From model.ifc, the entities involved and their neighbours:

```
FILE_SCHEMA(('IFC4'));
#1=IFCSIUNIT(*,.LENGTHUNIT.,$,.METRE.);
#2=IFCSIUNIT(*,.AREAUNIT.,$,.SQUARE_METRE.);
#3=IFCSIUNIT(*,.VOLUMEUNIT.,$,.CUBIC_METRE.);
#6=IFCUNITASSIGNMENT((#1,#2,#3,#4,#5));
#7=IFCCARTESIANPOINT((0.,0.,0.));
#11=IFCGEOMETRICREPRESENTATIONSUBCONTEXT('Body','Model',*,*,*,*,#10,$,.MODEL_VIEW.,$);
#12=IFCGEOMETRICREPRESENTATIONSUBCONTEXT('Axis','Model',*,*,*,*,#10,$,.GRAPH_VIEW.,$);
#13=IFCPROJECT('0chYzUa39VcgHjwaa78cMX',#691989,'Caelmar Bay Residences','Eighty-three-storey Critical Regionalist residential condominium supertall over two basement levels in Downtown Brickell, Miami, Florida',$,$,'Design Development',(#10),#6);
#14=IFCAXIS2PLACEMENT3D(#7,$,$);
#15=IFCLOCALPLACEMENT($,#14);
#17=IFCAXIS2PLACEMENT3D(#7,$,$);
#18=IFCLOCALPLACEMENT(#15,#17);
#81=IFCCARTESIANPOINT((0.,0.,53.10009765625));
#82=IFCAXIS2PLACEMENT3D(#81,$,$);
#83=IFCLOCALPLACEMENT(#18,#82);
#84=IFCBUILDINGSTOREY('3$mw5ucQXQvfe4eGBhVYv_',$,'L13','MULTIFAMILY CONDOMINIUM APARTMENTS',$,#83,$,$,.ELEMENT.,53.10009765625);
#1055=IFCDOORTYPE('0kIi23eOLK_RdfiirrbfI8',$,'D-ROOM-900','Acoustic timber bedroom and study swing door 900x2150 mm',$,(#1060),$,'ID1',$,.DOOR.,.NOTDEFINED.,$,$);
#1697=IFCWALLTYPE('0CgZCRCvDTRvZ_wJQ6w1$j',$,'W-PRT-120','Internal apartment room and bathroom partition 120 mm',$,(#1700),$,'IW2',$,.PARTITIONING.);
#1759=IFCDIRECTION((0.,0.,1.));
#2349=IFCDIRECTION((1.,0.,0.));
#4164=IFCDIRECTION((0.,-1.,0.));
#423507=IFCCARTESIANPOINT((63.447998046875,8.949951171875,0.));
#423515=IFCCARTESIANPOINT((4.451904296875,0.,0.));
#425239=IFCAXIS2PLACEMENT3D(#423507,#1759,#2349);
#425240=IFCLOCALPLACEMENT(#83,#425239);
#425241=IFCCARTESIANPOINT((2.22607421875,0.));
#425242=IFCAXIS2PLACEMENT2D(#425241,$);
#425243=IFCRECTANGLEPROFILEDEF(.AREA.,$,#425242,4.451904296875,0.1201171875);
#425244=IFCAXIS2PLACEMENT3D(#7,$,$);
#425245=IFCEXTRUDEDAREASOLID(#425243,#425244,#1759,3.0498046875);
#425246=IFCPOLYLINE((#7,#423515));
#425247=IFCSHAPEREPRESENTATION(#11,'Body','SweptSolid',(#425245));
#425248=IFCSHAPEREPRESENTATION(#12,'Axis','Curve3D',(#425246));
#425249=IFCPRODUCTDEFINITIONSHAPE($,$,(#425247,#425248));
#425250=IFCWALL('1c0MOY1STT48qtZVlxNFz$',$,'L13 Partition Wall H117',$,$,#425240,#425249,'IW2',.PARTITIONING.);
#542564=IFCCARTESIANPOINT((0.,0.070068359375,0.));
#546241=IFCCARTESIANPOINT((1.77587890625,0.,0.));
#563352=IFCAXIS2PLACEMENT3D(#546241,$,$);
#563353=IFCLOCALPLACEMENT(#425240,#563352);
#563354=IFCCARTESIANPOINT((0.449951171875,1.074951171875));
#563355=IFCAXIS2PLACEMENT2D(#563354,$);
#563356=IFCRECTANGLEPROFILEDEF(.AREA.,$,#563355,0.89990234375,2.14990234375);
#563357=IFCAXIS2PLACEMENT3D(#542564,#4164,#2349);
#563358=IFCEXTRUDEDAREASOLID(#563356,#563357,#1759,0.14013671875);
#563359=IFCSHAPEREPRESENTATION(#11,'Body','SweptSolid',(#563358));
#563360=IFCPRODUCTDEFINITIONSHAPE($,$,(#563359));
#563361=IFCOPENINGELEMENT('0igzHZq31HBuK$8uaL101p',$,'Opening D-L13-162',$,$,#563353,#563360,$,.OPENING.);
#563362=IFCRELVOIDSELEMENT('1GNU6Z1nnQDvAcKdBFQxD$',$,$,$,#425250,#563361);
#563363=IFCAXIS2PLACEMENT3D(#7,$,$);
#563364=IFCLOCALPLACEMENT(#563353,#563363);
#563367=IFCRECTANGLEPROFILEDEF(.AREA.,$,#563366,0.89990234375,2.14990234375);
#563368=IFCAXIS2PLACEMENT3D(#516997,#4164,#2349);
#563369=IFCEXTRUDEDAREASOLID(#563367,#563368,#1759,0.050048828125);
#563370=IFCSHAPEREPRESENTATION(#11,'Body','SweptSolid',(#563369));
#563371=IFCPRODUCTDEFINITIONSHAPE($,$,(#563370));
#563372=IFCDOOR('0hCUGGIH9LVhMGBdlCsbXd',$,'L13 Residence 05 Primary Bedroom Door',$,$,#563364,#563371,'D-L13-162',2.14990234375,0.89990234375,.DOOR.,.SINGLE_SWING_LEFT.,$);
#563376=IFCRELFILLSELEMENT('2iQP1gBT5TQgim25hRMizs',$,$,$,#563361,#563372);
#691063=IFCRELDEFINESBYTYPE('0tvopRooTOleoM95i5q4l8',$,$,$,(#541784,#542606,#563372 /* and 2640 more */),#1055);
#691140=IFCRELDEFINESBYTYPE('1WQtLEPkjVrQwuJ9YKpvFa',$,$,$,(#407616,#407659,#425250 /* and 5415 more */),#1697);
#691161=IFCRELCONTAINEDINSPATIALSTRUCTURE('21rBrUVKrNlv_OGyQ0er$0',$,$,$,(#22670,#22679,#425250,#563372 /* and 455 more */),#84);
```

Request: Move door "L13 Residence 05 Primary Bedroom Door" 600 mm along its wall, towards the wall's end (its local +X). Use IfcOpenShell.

```python
import ifcopenshell
import ifcopenshell.api.geometry
import ifcopenshell.util.placement
import ifcopenshell.util.unit

model = ifcopenshell.open("model.ifc")
unit_scale = ifcopenshell.util.unit.calculate_unit_scale(model)

door = model.by_guid("0hCUGGIH9LVhMGBdlCsbXd")
opening = door.FillsVoids[0].RelatingOpeningElement
wall = opening.VoidsElements[0].RelatingBuildingElement

wall_matrix = ifcopenshell.util.placement.get_local_placement(wall.ObjectPlacement)
shift = wall_matrix[:3, 0] * 0.6 / unit_scale
before = ifcopenshell.util.placement.get_local_placement(door.ObjectPlacement)[:3, 3].copy()

# The door is placed relative to its opening, so it follows when the opening moves.
matrix = ifcopenshell.util.placement.get_local_placement(opening.ObjectPlacement)
matrix[:3, 3] += shift
ifcopenshell.api.geometry.edit_object_placement(
    model, product=opening, matrix=matrix, is_si=False, should_transform_children=True
)

after = ifcopenshell.util.placement.get_local_placement(door.ObjectPlacement)[:3, 3]
print("door moved by", (after - before).round(3) + 0.0)

model.write("model_rev.ifc")
```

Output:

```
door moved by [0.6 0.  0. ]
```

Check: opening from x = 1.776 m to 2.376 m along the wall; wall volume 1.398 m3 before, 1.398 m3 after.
